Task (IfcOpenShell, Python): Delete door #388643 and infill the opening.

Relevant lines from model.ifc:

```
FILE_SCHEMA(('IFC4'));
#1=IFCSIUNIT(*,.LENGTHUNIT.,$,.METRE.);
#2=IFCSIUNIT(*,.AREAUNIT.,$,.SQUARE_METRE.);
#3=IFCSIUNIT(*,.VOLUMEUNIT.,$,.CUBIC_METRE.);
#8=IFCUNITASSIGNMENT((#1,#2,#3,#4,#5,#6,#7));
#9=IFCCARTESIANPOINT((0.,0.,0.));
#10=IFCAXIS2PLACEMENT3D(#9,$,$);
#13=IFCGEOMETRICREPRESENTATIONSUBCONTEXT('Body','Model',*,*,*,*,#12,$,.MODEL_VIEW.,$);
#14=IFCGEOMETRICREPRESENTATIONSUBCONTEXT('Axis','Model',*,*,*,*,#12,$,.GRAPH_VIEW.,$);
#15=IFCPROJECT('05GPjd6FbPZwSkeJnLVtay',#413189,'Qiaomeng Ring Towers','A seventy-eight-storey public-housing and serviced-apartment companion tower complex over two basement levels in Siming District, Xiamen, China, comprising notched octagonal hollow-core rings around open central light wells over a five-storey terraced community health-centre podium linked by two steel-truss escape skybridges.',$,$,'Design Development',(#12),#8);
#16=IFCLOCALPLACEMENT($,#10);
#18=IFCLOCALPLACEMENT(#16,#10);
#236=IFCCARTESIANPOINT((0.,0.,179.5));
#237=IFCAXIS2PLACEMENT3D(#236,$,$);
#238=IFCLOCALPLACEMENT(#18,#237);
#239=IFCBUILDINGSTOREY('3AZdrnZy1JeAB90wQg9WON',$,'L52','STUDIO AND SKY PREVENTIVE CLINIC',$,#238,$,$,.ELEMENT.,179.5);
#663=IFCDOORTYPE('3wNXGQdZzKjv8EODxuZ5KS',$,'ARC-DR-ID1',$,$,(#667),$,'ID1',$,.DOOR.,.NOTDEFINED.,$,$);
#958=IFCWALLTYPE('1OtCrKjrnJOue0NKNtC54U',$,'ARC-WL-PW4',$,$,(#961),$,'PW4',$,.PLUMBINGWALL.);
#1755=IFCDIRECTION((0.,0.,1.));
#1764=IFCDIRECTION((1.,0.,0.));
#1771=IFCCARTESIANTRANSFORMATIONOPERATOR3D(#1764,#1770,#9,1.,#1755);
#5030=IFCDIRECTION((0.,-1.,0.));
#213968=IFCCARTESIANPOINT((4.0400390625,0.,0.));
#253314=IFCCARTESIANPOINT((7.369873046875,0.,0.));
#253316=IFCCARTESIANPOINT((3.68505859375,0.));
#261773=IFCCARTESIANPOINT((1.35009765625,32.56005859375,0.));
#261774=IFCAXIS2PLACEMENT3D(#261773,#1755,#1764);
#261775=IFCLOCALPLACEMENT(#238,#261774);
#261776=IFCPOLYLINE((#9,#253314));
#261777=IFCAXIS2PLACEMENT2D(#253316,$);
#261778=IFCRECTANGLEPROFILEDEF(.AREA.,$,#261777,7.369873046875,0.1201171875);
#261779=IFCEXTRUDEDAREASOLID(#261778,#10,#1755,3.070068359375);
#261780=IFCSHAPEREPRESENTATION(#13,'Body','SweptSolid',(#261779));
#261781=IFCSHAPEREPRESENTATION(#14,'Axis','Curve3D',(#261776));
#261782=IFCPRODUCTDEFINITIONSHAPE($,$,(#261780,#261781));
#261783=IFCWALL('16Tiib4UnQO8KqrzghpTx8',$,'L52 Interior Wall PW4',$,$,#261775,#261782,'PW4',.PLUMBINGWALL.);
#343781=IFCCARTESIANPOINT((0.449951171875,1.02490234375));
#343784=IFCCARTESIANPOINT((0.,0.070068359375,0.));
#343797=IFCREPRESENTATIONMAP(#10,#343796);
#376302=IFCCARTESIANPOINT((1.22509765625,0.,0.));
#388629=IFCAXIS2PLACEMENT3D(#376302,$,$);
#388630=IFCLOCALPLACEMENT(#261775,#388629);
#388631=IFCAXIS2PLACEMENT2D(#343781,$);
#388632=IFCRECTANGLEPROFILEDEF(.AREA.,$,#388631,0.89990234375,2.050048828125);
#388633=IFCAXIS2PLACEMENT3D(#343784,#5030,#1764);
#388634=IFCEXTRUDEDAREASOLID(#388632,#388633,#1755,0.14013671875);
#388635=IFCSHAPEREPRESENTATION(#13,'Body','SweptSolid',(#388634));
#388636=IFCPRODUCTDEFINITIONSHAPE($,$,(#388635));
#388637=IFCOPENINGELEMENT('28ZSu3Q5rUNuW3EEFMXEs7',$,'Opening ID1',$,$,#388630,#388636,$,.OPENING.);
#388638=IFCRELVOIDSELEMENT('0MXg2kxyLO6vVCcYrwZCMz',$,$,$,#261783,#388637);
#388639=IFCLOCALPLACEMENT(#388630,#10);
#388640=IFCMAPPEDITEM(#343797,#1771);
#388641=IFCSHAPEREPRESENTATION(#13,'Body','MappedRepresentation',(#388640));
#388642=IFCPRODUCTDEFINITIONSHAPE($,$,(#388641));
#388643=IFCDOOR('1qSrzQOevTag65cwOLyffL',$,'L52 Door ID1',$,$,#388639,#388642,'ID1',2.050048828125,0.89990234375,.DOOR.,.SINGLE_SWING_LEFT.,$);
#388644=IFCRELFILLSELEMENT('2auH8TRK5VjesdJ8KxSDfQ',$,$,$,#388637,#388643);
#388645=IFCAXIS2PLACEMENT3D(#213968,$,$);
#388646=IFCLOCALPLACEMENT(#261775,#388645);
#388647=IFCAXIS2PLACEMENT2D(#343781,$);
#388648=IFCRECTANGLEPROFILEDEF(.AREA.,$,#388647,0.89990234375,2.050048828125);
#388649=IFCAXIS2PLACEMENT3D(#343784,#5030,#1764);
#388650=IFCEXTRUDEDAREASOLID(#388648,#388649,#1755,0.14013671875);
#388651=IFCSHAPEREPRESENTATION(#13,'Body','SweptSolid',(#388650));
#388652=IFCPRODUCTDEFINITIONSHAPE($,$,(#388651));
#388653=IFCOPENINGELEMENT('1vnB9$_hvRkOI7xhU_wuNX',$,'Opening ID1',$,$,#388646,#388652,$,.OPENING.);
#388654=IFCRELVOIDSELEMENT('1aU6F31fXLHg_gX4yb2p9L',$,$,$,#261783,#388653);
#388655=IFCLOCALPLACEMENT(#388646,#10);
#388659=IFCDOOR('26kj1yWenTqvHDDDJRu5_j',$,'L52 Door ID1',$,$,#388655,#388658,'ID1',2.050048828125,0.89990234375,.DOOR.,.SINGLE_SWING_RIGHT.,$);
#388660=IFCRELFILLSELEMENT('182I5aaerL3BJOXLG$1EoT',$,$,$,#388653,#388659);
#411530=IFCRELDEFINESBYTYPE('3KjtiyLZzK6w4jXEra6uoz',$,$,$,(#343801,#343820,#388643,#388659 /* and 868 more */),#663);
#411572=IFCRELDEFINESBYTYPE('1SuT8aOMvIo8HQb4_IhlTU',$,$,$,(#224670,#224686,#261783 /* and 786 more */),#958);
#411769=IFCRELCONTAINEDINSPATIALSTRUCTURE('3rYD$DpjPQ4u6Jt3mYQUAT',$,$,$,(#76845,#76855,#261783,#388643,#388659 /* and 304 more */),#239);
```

```python
import ifcopenshell
import ifcopenshell.api.feature
import ifcopenshell.api.root
import ifcopenshell.geom
import ifcopenshell.util.shape

model = ifcopenshell.open("model.ifc")
settings = ifcopenshell.geom.settings()


def volume(element):
    """Net volume in cubic metres, openings subtracted."""
    shape = ifcopenshell.geom.create_shape(settings, element)
    return ifcopenshell.util.shape.get_volume(shape.geometry)


door = model.by_id(388643)
opening = door.FillsVoids[0].RelatingOpeningElement
wall = opening.VoidsElements[0].RelatingBuildingElement
before = volume(wall)

ifcopenshell.api.root.remove_product(model, product=door)
ifcopenshell.api.feature.remove_feature(model, feature=opening)

after = volume(wall)

print(f"wall volume {before:.3f} -> {after:.3f} m3")

model.write("model_v2.ifc")
```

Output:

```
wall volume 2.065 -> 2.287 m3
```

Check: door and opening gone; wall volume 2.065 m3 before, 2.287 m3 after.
